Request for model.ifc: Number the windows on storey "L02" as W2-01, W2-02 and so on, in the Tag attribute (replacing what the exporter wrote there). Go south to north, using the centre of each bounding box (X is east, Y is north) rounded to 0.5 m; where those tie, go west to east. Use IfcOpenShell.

First a look at what the model holds.

```python
import ifcopenshell
import ifcopenshell.util.element
import ifcopenshell.util.placement

model = ifcopenshell.open("model.ifc")
print(model.schema)
storey = next(s for s in model.by_type("IfcBuildingStorey") if s.Name == "L02")
windows = [e for e in ifcopenshell.util.element.get_decomposition(storey) if e.is_a("IfcWindow")]
for e in sorted(windows, key=lambda e: e.id()):
    origin = ifcopenshell.util.placement.get_local_placement(e.ObjectPlacement)[:3, 3]
    print(e.id(), e.Tag, e.Name, origin.round(2) + 0.0, sep=" | ")
```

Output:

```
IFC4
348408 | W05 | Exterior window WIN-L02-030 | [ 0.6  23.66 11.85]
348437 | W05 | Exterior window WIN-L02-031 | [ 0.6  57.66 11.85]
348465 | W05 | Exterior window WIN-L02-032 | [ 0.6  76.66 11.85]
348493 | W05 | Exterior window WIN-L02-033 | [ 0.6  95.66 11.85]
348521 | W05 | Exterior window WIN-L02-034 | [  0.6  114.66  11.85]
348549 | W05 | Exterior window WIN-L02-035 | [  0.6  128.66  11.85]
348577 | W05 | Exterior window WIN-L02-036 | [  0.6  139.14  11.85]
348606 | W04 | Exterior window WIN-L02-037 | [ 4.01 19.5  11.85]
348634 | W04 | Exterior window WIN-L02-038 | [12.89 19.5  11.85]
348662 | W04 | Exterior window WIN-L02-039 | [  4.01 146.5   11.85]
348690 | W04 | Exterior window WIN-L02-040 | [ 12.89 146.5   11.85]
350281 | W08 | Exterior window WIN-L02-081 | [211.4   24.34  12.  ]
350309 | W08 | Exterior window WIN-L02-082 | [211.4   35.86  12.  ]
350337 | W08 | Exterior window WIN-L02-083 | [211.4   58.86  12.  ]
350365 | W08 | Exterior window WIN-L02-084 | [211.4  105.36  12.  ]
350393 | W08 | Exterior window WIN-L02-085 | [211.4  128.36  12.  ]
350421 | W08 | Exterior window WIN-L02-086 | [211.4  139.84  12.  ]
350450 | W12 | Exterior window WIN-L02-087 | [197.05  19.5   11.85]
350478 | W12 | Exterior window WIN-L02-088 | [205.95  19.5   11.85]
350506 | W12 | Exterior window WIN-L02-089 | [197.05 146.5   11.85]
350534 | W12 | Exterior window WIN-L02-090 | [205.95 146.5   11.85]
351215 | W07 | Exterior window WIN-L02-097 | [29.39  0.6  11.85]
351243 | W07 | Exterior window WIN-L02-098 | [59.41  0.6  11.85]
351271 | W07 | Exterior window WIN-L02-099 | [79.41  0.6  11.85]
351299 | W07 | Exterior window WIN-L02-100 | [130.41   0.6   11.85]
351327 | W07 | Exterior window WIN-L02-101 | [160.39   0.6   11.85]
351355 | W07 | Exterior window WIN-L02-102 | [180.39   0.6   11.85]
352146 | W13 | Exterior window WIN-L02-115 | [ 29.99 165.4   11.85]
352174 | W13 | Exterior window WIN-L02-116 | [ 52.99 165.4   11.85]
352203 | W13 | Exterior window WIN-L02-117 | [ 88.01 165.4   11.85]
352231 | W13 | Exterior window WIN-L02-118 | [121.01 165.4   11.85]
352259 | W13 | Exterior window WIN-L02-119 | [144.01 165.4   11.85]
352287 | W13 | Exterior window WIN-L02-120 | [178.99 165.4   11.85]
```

```python
import ifcopenshell
import ifcopenshell.geom
import ifcopenshell.util.element
import ifcopenshell.util.shape

model = ifcopenshell.open("model.ifc")
settings = ifcopenshell.geom.settings()
settings.set("use-world-coords", True)


def centre(element):
    shape = ifcopenshell.geom.create_shape(settings, element)
    return ifcopenshell.util.shape.get_bbox_centroid(shape.geometry)


storey = next(s for s in model.by_type("IfcBuildingStorey") if s.Name == "L02")
windows = [e for e in ifcopenshell.util.element.get_decomposition(storey) if e.is_a("IfcWindow")]

# Insertion points can sit at a corner or the storey origin, so sort by the geometry (in metres).
centres = {e: centre(e) for e in windows}
windows.sort(key=lambda e: (round(centres[e][1] / 0.5), centres[e][0]))

for i, e in enumerate(windows, start=1):
    number = f"W2-{i:02d}"
    e.Tag = number
    print(e.id(), number)

model.write("model_rev.ifc")
```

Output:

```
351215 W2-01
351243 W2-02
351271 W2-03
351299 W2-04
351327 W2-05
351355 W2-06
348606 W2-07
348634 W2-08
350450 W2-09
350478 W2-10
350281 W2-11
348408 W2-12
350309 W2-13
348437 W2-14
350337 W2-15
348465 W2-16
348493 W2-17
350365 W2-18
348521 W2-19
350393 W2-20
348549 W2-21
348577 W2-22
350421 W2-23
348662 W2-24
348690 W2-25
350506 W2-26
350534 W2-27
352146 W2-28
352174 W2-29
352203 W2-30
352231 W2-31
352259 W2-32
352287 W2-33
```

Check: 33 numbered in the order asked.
